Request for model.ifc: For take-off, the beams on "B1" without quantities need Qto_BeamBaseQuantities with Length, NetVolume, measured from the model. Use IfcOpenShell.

First a look at what the model holds.

```python
import ifcopenshell
import ifcopenshell.util.element
import ifcopenshell.util.unit

model = ifcopenshell.open("model.ifc")
print(model.schema)
for unit_type in ("LENGTHUNIT", "AREAUNIT", "VOLUMEUNIT"):
    print(unit_type, ifcopenshell.util.unit.calculate_unit_scale(model, unit_type))
storey = next(s for s in model.by_type("IfcBuildingStorey") if s.Name == "B1")
beams = [e for e in ifcopenshell.util.element.get_decomposition(storey) if e.is_a("IfcBeam")]
for e in sorted(beams, key=lambda e: e.id()):
    print(e.id(), e.is_a(), e.Name, list(ifcopenshell.util.element.get_psets(e, qtos_only=True)), sep=" | ")
```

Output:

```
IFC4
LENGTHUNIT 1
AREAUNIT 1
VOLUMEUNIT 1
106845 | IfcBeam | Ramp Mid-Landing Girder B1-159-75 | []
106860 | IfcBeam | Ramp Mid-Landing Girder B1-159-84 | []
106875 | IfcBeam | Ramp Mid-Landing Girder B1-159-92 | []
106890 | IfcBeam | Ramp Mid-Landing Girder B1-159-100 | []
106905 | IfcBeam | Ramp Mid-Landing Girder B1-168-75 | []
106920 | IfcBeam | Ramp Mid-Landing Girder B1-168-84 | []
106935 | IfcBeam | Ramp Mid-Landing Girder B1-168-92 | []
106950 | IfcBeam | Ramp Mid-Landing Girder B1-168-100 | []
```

```python
import ifcopenshell
import ifcopenshell.api.pset
import ifcopenshell.geom
import ifcopenshell.util.element
import ifcopenshell.util.shape
import ifcopenshell.util.unit

model = ifcopenshell.open("model.ifc")
unit_scale = ifcopenshell.util.unit.calculate_unit_scale(model)
volume_scale = ifcopenshell.util.unit.calculate_unit_scale(model, "VOLUMEUNIT")
settings = ifcopenshell.geom.settings()

storey = next(s for s in model.by_type("IfcBuildingStorey") if s.Name == "B1")
beams = [e for e in ifcopenshell.util.element.get_decomposition(storey) if e.is_a("IfcBeam")]

for e in sorted(beams, key=lambda e: e.id()):
    if ifcopenshell.util.element.get_psets(e, qtos_only=True, should_inherit=False):
        continue
    # Geometry comes back in metres, in the element's own axes.
    shape = ifcopenshell.geom.create_shape(settings, e)
    values = {
        "Length": ifcopenshell.util.shape.get_max_xyz(shape.geometry) / unit_scale,
        "NetVolume": ifcopenshell.util.shape.get_volume(shape.geometry) / volume_scale,
    }
    qto = ifcopenshell.api.pset.add_qto(model, product=e, name="Qto_BeamBaseQuantities")
    ifcopenshell.api.pset.edit_qto(model, qto=qto, properties=values)
    print(e.id(), {k: round(v, 3) for k, v in values.items()})

model.write("model_v2.ifc")
```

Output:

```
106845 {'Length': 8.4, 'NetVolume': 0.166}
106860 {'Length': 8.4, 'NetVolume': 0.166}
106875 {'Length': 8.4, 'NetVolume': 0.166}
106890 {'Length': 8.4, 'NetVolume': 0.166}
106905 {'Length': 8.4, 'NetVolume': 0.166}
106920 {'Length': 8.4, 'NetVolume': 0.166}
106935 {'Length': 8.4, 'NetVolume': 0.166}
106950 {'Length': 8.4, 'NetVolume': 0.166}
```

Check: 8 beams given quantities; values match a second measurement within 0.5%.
